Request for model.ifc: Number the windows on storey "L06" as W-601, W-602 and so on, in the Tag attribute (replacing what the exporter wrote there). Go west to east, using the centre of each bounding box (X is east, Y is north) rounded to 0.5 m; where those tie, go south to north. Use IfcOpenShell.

First a look at what the model holds.

```python
import ifcopenshell
import ifcopenshell.util.element
import ifcopenshell.util.placement

model = ifcopenshell.open("model.ifc")
print(model.schema)
storey = next(s for s in model.by_type("IfcBuildingStorey") if s.Name == "L06")
windows = [e for e in ifcopenshell.util.element.get_decomposition(storey) if e.is_a("IfcWindow")]
for e in sorted(windows, key=lambda e: e.id()):
    origin = ifcopenshell.util.placement.get_local_placement(e.ObjectPlacement)[:3, 3]
    print(e.id(), e.Tag, e.Name, origin.round(2) + 0.0, sep=" | ")
```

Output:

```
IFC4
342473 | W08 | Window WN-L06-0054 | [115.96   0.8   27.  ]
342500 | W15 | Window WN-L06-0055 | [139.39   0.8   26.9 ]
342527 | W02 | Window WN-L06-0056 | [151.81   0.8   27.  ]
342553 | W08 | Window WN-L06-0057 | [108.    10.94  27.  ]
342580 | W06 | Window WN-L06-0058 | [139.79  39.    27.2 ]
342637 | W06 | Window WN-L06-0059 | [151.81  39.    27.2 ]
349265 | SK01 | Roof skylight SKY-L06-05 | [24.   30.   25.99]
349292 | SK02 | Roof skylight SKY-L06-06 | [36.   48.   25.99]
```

```python
import ifcopenshell
import ifcopenshell.geom
import ifcopenshell.util.element
import ifcopenshell.util.shape

model = ifcopenshell.open("model.ifc")
settings = ifcopenshell.geom.settings()
settings.set("use-world-coords", True)


def centre(element):
    shape = ifcopenshell.geom.create_shape(settings, element)
    return ifcopenshell.util.shape.get_bbox_centroid(shape.geometry)


storey = next(s for s in model.by_type("IfcBuildingStorey") if s.Name == "L06")
windows = [e for e in ifcopenshell.util.element.get_decomposition(storey) if e.is_a("IfcWindow")]

# Insertion points can sit at a corner or the storey origin, so sort by the geometry (in metres).
centres = {e: centre(e) for e in windows}
windows.sort(key=lambda e: (round(centres[e][0] / 0.5), centres[e][1]))

for i, e in enumerate(windows, start=1):
    number = f"W-6{i:02d}"
    e.Tag = number
    print(e.id(), number)

model.write("model_v2.ifc")
```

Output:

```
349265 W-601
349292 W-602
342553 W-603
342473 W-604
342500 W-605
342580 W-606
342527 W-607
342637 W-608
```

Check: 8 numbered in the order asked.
